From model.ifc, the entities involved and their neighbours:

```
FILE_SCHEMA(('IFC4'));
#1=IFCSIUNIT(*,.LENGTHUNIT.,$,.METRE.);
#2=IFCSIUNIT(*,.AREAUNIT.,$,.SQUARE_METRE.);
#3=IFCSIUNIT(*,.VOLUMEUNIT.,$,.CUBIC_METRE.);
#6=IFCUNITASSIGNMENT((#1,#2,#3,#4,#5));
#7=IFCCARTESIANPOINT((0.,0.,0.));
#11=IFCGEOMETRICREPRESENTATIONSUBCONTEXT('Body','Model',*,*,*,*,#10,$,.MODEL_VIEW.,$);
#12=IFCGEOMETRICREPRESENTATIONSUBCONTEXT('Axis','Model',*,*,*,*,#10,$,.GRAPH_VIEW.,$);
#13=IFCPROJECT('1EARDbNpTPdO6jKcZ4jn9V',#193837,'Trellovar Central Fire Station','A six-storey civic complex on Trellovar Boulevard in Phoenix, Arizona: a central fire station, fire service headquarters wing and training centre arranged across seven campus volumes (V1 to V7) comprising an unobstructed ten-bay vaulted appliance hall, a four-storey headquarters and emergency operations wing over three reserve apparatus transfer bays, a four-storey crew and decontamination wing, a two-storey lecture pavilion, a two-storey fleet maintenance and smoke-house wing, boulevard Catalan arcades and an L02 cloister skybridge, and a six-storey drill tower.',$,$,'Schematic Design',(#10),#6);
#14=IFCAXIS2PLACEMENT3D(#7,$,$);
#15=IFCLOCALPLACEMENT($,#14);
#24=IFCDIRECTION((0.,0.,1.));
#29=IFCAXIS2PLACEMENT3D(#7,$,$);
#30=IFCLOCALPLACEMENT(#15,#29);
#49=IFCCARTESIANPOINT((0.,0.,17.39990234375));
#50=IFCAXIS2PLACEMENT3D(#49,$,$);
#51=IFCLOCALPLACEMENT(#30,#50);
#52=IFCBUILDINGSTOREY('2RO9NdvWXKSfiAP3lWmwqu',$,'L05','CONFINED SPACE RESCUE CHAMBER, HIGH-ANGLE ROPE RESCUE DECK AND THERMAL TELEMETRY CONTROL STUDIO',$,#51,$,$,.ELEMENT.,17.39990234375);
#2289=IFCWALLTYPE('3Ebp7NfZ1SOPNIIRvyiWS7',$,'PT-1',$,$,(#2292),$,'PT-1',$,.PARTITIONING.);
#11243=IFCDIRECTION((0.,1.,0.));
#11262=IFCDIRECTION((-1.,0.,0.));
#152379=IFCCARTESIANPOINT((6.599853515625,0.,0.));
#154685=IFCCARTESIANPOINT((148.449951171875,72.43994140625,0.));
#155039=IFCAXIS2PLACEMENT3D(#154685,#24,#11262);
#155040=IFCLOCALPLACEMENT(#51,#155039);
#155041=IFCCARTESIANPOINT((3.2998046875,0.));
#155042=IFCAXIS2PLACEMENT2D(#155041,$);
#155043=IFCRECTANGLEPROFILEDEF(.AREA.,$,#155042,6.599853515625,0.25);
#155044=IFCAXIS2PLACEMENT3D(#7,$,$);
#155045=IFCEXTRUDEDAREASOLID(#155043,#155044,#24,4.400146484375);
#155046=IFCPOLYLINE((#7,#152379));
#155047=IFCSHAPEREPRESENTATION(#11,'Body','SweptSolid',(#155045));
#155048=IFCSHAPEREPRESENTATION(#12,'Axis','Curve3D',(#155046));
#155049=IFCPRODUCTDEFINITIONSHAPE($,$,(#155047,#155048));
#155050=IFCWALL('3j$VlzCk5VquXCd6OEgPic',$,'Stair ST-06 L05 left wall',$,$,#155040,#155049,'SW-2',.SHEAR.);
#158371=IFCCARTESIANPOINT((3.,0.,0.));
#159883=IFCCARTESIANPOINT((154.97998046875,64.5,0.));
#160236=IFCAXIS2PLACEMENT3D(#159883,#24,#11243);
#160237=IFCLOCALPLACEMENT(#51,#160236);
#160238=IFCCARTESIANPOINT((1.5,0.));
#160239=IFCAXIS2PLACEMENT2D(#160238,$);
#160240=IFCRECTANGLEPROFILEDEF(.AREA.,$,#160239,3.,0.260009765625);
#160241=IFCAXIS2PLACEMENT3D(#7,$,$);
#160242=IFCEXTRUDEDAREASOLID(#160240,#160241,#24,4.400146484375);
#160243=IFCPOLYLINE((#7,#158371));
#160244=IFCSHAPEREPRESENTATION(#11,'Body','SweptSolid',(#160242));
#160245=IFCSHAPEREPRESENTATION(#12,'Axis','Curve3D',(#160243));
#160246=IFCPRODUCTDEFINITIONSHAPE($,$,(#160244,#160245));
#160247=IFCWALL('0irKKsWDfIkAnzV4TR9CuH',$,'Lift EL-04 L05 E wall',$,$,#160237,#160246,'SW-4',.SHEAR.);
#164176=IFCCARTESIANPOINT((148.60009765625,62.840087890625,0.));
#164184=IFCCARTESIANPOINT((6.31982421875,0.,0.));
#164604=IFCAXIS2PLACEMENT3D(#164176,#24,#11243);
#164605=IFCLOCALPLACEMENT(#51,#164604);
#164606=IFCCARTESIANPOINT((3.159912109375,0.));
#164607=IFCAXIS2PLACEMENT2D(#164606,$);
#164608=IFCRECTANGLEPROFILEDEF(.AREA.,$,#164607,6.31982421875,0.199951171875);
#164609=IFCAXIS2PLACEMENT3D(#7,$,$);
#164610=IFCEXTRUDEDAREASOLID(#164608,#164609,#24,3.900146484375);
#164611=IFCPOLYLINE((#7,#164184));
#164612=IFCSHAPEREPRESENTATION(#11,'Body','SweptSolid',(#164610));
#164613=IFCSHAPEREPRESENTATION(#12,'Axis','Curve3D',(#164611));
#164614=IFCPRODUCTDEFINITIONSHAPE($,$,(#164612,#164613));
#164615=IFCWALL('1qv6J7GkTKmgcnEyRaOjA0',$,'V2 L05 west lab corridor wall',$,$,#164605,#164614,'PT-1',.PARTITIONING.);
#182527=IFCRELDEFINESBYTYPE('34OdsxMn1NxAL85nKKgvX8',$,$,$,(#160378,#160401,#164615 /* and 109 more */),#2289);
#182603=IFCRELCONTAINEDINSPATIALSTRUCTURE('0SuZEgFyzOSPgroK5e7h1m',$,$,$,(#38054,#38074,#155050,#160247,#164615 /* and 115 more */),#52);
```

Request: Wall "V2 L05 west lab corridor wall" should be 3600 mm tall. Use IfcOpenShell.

```python
import ifcopenshell
import ifcopenshell.geom
import ifcopenshell.util.representation
import ifcopenshell.util.shape

model = ifcopenshell.open("model.ifc")
settings = ifcopenshell.geom.settings()


def volume(element):
    """Net volume in cubic metres, openings subtracted."""
    shape = ifcopenshell.geom.create_shape(settings, element)
    return ifcopenshell.util.shape.get_volume(shape.geometry)


wall = model.by_id(164615)
before = volume(wall)

body = ifcopenshell.util.representation.get_representation(wall, "Model", "Body")
solid = body.Items[0]
old_height = solid.Depth
solid.Depth = 3.6
after = volume(wall)

print(f"height {old_height:g} -> {solid.Depth:g}, volume {before:.3f} -> {after:.3f} m3")

model.write("model_rev.ifc")
```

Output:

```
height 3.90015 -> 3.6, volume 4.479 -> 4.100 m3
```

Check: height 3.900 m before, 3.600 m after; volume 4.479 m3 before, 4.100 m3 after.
